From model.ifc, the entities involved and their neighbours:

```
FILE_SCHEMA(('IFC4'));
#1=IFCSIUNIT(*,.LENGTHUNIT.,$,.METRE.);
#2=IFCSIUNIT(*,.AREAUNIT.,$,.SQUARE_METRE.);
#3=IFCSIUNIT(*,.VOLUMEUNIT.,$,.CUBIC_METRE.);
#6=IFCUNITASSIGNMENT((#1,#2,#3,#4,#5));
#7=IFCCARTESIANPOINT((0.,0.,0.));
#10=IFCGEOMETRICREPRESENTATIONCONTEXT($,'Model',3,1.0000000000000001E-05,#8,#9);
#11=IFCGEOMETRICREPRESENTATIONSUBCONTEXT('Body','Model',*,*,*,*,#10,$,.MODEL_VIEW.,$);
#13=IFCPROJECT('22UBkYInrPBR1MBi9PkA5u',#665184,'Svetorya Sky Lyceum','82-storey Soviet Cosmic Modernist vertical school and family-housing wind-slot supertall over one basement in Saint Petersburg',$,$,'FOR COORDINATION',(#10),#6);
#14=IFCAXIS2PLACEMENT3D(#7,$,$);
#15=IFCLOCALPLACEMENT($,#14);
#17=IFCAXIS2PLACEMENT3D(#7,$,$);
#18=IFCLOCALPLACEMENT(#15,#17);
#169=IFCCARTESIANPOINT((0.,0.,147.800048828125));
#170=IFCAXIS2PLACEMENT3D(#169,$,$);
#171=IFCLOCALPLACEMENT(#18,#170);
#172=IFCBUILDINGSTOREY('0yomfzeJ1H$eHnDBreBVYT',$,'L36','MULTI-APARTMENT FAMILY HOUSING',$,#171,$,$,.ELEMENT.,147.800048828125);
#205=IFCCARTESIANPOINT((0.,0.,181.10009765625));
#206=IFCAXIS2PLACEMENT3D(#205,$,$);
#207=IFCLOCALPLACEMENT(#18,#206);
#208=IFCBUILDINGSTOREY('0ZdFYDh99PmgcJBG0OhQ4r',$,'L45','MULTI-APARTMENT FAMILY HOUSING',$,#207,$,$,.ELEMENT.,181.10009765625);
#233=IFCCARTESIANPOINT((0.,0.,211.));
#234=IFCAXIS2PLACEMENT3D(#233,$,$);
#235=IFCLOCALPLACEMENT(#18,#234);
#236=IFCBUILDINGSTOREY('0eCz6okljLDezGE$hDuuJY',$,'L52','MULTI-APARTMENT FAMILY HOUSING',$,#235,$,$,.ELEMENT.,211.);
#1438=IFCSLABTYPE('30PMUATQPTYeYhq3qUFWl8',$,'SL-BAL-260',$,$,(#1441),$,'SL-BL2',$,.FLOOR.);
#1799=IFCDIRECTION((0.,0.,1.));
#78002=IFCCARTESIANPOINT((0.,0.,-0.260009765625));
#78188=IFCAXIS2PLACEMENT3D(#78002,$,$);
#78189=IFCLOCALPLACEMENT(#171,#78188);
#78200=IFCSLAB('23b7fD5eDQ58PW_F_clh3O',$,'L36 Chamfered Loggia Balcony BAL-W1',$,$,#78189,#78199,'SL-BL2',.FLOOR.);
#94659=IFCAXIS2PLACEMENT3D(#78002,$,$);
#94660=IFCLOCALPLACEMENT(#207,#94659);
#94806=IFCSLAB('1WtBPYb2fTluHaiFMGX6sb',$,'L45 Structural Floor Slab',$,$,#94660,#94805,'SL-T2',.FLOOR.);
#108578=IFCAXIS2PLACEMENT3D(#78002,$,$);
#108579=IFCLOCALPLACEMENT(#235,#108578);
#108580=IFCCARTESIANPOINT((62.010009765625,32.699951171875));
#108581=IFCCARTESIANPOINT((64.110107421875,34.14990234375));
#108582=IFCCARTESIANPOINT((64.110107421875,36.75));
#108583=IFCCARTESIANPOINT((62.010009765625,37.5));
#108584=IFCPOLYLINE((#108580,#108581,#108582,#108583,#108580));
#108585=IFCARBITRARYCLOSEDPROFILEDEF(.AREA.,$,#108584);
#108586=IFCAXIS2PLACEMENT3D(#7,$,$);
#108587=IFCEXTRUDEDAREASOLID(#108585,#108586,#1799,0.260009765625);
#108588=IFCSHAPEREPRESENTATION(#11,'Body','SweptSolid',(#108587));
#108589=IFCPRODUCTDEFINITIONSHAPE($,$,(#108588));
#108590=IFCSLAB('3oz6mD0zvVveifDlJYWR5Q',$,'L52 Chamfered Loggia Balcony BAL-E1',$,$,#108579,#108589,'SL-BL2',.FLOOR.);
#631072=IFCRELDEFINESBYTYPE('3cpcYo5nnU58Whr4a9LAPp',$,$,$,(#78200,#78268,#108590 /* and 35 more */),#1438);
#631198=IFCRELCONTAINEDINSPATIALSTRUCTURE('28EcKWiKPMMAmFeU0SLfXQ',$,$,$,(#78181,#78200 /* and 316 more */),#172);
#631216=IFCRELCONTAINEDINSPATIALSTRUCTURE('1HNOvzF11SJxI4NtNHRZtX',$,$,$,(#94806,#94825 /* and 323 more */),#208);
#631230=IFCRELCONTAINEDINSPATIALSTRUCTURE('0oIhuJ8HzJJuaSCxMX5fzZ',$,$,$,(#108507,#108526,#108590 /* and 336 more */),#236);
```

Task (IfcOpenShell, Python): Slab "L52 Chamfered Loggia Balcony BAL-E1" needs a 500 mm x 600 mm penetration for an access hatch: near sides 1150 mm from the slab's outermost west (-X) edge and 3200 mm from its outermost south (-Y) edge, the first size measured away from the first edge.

```python
import numpy as np
import ifcopenshell
import ifcopenshell.api.feature
import ifcopenshell.api.geometry
import ifcopenshell.api.root
import ifcopenshell.geom
import ifcopenshell.util.placement
import ifcopenshell.util.representation
import ifcopenshell.util.shape
import ifcopenshell.util.unit

model = ifcopenshell.open("model.ifc")
unit_scale = ifcopenshell.util.unit.calculate_unit_scale(model)
settings = ifcopenshell.geom.settings()


def volume(element):
    """Net volume in cubic metres, openings subtracted."""
    shape = ifcopenshell.geom.create_shape(settings, element)
    return ifcopenshell.util.shape.get_volume(shape.geometry)


slab = model.by_id(108590)
before = volume(slab)

# Extent in the slab's own axes, in metres. The edges named are its -X and -Y sides.
slab_shape = ifcopenshell.geom.create_shape(settings, slab)
vertices = ifcopenshell.util.shape.get_vertices(slab_shape.geometry)
x_min, y_min, bottom = vertices.min(axis=0)
top = vertices[:, 2].max()

opening = ifcopenshell.api.root.create_entity(model, ifc_class="IfcOpeningElement", name="Access hatch opening", predefined_type="OPENING")
context = ifcopenshell.util.representation.get_context(model, "Model", "Body", "MODEL_VIEW")
width, depth = 0.5, 0.6
outline = [(0.0, 0.0), (width, 0.0), (width, depth), (0.0, depth), (0.0, 0.0)]
# Overshoot both faces by 50 mm so the cut is clean.
shape = ifcopenshell.api.geometry.add_slab_representation(
    model, context=context, depth=top - bottom + 0.1, polyline=outline
)
ifcopenshell.api.geometry.assign_representation(model, product=opening, representation=shape)

matrix = ifcopenshell.util.placement.get_local_placement(slab.ObjectPlacement)
matrix[:, 3] = matrix @ np.append(np.array([x_min + 1.15, y_min + 3.2, bottom - 0.05]) / unit_scale, 1.0)
ifcopenshell.api.geometry.edit_object_placement(model, product=opening, matrix=matrix, is_si=False)
ifcopenshell.api.feature.add_feature(model, feature=opening, element=slab)

after = volume(slab)

print(f"slab volume {before:.3f} -> {after:.3f} m3")

model.write("model_rev.ifc")
```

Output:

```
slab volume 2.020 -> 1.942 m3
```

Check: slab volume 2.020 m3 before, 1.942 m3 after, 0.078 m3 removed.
